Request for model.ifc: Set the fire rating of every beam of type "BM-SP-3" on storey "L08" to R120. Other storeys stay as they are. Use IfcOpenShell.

First a look at what the model holds.

```python
import ifcopenshell
import ifcopenshell.util.element

model = ifcopenshell.open("model.ifc")
print(model.schema)
storey = next(s for s in model.by_type("IfcBuildingStorey") if s.Name == "L08")
beams = [e for e in ifcopenshell.util.element.get_decomposition(storey) if e.is_a("IfcBeam")]
seen = {}
for e in beams:
    element_type = ifcopenshell.util.element.get_type(e)
    key = (element_type.Name if element_type != e and element_type else None, ifcopenshell.util.element.get_pset(e, "Pset_BeamCommon", "FireRating"))
    seen[key] = seen.get(key, 0) + 1
for (name, value), count in sorted(seen.items(), key=str):
    print(count, "x", name, "|", value)
```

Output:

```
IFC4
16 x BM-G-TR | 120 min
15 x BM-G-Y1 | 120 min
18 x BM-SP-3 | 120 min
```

```python
import ifcopenshell
import ifcopenshell.api.pset
import ifcopenshell.util.element

model = ifcopenshell.open("model.ifc")

storey = next(s for s in model.by_type("IfcBuildingStorey") if s.Name == "L08")
beams = [e for e in ifcopenshell.util.element.get_decomposition(storey) if e.is_a("IfcBeam")]

count = 0
for e in beams:
    element_type = ifcopenshell.util.element.get_type(e)
    if element_type in (None, e) or element_type.Name != "BM-SP-3":
        continue
    # add_pset returns the element's existing set when there is one.
    pset = ifcopenshell.api.pset.add_pset(model, product=e, name="Pset_BeamCommon")
    ifcopenshell.api.pset.edit_pset(model, pset=pset, properties={"FireRating": "R120"})
    count += 1

print(count, "beams updated")

model.write("model_edited.ifc")
```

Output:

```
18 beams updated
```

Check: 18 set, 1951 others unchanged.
